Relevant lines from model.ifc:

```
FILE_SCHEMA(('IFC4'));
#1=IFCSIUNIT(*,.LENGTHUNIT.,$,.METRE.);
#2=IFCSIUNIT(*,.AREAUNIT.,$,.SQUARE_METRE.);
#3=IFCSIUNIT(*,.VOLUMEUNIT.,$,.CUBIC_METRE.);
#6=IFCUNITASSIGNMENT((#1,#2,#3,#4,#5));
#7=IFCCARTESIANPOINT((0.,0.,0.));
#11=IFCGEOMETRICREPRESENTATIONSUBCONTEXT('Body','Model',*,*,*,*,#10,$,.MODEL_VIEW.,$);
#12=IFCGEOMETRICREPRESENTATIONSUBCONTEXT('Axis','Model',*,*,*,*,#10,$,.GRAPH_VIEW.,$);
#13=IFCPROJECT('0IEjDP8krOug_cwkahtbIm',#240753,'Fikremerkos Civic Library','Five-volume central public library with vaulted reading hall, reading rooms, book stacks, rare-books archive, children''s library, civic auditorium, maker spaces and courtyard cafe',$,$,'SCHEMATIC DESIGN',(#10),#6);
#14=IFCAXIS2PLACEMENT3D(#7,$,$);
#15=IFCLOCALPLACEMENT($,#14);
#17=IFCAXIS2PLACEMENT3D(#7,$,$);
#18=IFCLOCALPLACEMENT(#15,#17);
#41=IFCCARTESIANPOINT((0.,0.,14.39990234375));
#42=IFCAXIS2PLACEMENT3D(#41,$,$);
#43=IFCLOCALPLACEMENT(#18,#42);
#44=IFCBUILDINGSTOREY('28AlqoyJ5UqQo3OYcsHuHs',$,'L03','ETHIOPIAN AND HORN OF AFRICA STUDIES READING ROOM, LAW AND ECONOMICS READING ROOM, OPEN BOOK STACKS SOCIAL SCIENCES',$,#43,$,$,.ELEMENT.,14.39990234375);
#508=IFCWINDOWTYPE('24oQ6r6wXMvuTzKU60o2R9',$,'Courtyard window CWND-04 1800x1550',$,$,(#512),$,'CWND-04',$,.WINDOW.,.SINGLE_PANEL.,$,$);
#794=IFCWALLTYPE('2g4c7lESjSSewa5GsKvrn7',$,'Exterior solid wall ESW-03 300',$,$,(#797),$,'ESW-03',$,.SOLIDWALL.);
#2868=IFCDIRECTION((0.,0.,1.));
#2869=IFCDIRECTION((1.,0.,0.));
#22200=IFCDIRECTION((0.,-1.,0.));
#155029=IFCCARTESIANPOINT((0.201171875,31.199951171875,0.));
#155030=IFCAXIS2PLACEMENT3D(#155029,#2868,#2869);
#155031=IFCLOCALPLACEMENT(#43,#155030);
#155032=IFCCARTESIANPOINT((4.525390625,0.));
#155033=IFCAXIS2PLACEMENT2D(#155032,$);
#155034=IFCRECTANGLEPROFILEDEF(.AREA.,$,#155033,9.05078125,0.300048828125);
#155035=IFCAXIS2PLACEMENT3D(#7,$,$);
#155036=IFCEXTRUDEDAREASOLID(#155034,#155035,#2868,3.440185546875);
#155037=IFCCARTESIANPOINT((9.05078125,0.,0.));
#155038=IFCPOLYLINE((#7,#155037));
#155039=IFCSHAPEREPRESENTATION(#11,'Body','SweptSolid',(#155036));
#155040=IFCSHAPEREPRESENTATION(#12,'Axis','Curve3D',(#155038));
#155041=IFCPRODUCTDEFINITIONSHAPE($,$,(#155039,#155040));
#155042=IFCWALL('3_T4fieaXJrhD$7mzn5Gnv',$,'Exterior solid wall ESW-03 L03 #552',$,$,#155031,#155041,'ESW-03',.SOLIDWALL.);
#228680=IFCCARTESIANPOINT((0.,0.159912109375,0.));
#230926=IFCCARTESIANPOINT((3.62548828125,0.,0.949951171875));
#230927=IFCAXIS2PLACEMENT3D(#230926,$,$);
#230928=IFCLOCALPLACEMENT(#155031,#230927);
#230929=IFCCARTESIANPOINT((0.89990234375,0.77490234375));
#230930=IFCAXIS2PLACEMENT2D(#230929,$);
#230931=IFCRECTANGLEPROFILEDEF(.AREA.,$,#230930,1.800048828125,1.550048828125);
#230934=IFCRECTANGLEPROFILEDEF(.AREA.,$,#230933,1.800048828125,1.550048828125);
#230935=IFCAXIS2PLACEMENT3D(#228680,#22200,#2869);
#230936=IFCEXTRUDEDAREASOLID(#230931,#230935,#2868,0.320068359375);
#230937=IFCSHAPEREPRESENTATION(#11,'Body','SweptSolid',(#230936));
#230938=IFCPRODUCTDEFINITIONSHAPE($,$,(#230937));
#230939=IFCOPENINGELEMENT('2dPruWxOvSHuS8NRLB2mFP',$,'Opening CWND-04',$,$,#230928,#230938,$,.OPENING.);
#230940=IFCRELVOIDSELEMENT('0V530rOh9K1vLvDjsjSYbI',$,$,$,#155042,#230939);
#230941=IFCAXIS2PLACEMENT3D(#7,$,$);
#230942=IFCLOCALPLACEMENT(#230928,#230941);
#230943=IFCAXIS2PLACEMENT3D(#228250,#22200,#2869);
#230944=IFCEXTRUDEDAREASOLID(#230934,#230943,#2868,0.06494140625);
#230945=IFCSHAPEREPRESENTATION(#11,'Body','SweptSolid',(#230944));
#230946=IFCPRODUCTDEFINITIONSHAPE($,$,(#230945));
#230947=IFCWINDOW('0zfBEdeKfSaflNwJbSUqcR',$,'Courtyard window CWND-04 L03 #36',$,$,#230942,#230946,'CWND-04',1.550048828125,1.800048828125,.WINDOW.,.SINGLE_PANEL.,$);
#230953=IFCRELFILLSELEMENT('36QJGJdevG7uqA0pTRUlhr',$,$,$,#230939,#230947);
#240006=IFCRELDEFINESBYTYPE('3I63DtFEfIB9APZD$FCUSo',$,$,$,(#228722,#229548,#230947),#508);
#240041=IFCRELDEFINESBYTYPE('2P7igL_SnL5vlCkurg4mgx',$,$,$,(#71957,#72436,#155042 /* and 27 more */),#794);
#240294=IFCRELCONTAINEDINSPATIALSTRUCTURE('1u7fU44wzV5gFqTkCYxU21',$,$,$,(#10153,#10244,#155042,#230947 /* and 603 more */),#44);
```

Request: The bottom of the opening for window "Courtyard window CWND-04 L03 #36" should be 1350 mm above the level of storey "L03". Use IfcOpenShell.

```python
import numpy as np
import ifcopenshell
import ifcopenshell.api.geometry
import ifcopenshell.geom
import ifcopenshell.util.element
import ifcopenshell.util.placement
import ifcopenshell.util.shape
import ifcopenshell.util.unit

model = ifcopenshell.open("model.ifc")
unit_scale = ifcopenshell.util.unit.calculate_unit_scale(model)

window = model.by_guid("0zfBEdeKfSaflNwJbSUqcR")
opening = window.FillsVoids[0].RelatingOpeningElement
storey = ifcopenshell.util.element.get_container(window, ifc_class="IfcBuildingStorey")
level = ifcopenshell.util.placement.get_local_placement(storey.ObjectPlacement)[2, 3]

# The opening's origin need not be at the sill, so measure its lowest point.
shape = ifcopenshell.geom.create_shape(ifcopenshell.geom.settings(), opening)
bottom = ifcopenshell.util.shape.get_shape_bottom_elevation(shape, shape.geometry) / unit_scale
dz = level + 1.35 - bottom

shift = np.array([0.0, 0.0, dz])
# The window is placed relative to its opening, so it follows when the opening moves.
matrix = ifcopenshell.util.placement.get_local_placement(opening.ObjectPlacement)
matrix[:3, 3] += shift
ifcopenshell.api.geometry.edit_object_placement(
    model, product=opening, matrix=matrix, is_si=False, should_transform_children=True
)

print(f"moved by {dz * unit_scale:+.3f} m")

model.write("model_rev.ifc")
```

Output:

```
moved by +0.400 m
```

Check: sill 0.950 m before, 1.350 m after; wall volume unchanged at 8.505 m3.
